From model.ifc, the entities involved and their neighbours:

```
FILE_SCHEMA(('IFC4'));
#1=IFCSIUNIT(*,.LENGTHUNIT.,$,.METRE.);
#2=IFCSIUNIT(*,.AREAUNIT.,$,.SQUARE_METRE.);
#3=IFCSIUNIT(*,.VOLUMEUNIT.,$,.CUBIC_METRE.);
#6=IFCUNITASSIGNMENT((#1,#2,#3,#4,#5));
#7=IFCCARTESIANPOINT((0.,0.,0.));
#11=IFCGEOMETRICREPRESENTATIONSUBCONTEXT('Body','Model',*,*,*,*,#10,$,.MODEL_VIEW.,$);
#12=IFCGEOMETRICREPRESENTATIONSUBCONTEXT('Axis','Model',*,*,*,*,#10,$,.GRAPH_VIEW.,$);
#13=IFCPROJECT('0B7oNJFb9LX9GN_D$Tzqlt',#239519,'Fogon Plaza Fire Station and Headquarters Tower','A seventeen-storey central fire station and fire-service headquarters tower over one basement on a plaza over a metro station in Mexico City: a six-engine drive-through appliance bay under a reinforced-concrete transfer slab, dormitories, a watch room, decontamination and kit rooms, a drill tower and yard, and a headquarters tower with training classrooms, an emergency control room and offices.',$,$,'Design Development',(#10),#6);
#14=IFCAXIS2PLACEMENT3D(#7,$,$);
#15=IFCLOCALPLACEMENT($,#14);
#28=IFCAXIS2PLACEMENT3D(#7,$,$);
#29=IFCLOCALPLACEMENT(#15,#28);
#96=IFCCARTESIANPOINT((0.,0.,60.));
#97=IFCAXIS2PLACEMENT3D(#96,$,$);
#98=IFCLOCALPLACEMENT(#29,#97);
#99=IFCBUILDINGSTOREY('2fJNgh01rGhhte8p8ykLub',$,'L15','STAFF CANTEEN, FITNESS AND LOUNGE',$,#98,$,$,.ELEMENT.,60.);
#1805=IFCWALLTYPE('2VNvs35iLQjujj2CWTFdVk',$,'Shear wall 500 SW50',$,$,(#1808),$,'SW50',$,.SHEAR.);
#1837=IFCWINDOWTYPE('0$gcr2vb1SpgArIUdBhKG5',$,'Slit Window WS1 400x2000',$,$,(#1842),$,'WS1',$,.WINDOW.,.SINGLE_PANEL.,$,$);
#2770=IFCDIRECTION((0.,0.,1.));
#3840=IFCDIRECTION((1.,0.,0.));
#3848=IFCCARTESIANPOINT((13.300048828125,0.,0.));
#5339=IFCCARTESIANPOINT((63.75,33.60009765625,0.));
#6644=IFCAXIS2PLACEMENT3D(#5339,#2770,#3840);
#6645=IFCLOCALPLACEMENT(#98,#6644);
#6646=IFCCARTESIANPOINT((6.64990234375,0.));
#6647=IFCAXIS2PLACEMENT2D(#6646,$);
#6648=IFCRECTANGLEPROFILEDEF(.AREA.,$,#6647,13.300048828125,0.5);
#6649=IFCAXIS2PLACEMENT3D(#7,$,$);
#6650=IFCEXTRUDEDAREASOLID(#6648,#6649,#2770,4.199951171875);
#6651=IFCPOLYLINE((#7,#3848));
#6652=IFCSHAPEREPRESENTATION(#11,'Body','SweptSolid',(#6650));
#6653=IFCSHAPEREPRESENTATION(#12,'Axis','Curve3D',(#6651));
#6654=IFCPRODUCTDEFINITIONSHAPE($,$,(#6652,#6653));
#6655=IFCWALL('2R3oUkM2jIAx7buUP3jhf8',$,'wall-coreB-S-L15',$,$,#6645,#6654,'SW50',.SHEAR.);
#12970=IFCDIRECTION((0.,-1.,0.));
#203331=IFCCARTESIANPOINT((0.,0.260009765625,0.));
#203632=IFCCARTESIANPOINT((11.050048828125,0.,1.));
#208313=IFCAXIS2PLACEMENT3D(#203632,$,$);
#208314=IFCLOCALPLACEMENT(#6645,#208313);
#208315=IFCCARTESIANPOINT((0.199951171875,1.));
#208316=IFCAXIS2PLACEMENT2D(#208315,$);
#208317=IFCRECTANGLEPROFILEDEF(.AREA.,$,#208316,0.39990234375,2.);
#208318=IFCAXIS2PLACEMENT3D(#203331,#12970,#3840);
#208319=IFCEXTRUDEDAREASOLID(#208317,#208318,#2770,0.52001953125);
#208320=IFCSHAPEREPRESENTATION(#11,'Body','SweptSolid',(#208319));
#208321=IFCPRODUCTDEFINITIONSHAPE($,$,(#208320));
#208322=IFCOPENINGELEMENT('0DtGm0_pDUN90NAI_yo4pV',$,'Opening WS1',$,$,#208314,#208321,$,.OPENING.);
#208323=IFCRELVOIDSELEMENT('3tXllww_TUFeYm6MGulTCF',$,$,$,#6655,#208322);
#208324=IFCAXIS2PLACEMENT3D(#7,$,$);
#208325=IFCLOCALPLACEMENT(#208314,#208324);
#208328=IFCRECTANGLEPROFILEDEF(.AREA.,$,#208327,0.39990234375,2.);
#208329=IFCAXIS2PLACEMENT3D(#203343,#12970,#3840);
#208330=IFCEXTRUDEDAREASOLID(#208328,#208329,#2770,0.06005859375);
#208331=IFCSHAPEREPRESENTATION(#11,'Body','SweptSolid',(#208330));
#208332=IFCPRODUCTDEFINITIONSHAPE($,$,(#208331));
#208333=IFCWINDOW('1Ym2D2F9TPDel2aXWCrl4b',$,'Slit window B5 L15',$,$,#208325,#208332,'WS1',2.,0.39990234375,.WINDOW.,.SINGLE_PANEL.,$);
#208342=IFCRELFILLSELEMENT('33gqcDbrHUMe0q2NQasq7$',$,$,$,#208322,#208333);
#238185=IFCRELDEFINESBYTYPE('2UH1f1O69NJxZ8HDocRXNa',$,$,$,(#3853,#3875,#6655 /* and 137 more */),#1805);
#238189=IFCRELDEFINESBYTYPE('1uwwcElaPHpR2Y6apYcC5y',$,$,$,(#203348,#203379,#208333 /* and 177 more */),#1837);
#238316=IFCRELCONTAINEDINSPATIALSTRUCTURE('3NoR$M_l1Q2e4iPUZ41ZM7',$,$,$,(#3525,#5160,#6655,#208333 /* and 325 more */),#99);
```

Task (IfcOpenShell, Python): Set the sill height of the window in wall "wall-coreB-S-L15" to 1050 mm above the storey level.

```python
import numpy as np
import ifcopenshell
import ifcopenshell.api.geometry
import ifcopenshell.geom
import ifcopenshell.util.element
import ifcopenshell.util.placement
import ifcopenshell.util.shape
import ifcopenshell.util.unit

model = ifcopenshell.open("model.ifc")
unit_scale = ifcopenshell.util.unit.calculate_unit_scale(model)

window = model.by_guid("1Ym2D2F9TPDel2aXWCrl4b")
opening = window.FillsVoids[0].RelatingOpeningElement
storey = ifcopenshell.util.element.get_container(window, ifc_class="IfcBuildingStorey")
level = ifcopenshell.util.placement.get_local_placement(storey.ObjectPlacement)[2, 3]

# The opening's origin need not be at the sill, so measure its lowest point.
shape = ifcopenshell.geom.create_shape(ifcopenshell.geom.settings(), opening)
bottom = ifcopenshell.util.shape.get_shape_bottom_elevation(shape, shape.geometry) / unit_scale
dz = level + 1.05 / unit_scale - bottom

shift = np.array([0.0, 0.0, dz])
# The window is placed relative to its opening, so it follows when the opening moves.
matrix = ifcopenshell.util.placement.get_local_placement(opening.ObjectPlacement)
matrix[:3, 3] += shift
ifcopenshell.api.geometry.edit_object_placement(
    model, product=opening, matrix=matrix, is_si=False, should_transform_children=True
)

print(f"moved by {dz * unit_scale:+.3f} m")

model.write("model_edited.ifc")
```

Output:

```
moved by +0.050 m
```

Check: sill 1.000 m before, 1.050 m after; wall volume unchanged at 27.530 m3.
